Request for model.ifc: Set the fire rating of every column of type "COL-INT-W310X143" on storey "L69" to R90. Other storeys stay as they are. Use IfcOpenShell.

First a look at what the model holds.

```python
import ifcopenshell
import ifcopenshell.util.element

model = ifcopenshell.open("model.ifc")
print(model.schema)
storey = next(s for s in model.by_type("IfcBuildingStorey") if s.Name == "L69")
columns = [e for e in ifcopenshell.util.element.get_decomposition(storey) if e.is_a("IfcColumn")]
seen = {}
for e in columns:
    element_type = ifcopenshell.util.element.get_type(e)
    key = (element_type.Name if element_type != e and element_type else None, ifcopenshell.util.element.get_pset(e, "Pset_ColumnCommon", "FireRating"))
    seen[key] = seen.get(key, 0) + 1
for (name, value), count in sorted(seen.items(), key=str):
    print(count, "x", name, "|", value)
```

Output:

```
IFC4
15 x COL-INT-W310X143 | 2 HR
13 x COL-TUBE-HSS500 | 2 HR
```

```python
import ifcopenshell
import ifcopenshell.api.pset
import ifcopenshell.util.element

model = ifcopenshell.open("model.ifc")

storey = next(s for s in model.by_type("IfcBuildingStorey") if s.Name == "L69")
columns = [e for e in ifcopenshell.util.element.get_decomposition(storey) if e.is_a("IfcColumn")]

count = 0
for e in columns:
    element_type = ifcopenshell.util.element.get_type(e)
    if element_type in (None, e) or element_type.Name != "COL-INT-W310X143":
        continue
    found = ifcopenshell.util.element.get_pset(e, "Pset_ColumnCommon", should_inherit=False)
    if found:
        pset = model.by_id(found["id"])
        if len(ifcopenshell.util.element.get_elements_by_pset(pset)) > 1:
            pset = ifcopenshell.api.pset.unshare_pset(model, products=[e], pset=pset)[0]
    else:
        pset = ifcopenshell.api.pset.add_pset(model, product=e, name="Pset_ColumnCommon")
    ifcopenshell.api.pset.edit_pset(model, pset=pset, properties={"FireRating": "R90"})
    count += 1

print(count, "columns updated")

model.write("model_edited.ifc")
```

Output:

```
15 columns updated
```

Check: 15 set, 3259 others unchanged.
